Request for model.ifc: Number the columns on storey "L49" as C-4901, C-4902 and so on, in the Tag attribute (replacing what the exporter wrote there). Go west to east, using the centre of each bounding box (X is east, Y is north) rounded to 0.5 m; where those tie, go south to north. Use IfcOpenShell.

First a look at what the model holds.

```python
import ifcopenshell
import ifcopenshell.util.element
import ifcopenshell.util.placement

model = ifcopenshell.open("model.ifc")
print(model.schema)
storey = next(s for s in model.by_type("IfcBuildingStorey") if s.Name == "L49")
columns = [e for e in ifcopenshell.util.element.get_decomposition(storey) if e.is_a("IfcColumn")]
for e in sorted(columns, key=lambda e: e.id()):
    origin = ifcopenshell.util.placement.get_local_placement(e.ObjectPlacement)[:3, 3]
    print(e.id(), e.Tag, e.Name, origin.round(2) + 0.0, sep=" | ")
```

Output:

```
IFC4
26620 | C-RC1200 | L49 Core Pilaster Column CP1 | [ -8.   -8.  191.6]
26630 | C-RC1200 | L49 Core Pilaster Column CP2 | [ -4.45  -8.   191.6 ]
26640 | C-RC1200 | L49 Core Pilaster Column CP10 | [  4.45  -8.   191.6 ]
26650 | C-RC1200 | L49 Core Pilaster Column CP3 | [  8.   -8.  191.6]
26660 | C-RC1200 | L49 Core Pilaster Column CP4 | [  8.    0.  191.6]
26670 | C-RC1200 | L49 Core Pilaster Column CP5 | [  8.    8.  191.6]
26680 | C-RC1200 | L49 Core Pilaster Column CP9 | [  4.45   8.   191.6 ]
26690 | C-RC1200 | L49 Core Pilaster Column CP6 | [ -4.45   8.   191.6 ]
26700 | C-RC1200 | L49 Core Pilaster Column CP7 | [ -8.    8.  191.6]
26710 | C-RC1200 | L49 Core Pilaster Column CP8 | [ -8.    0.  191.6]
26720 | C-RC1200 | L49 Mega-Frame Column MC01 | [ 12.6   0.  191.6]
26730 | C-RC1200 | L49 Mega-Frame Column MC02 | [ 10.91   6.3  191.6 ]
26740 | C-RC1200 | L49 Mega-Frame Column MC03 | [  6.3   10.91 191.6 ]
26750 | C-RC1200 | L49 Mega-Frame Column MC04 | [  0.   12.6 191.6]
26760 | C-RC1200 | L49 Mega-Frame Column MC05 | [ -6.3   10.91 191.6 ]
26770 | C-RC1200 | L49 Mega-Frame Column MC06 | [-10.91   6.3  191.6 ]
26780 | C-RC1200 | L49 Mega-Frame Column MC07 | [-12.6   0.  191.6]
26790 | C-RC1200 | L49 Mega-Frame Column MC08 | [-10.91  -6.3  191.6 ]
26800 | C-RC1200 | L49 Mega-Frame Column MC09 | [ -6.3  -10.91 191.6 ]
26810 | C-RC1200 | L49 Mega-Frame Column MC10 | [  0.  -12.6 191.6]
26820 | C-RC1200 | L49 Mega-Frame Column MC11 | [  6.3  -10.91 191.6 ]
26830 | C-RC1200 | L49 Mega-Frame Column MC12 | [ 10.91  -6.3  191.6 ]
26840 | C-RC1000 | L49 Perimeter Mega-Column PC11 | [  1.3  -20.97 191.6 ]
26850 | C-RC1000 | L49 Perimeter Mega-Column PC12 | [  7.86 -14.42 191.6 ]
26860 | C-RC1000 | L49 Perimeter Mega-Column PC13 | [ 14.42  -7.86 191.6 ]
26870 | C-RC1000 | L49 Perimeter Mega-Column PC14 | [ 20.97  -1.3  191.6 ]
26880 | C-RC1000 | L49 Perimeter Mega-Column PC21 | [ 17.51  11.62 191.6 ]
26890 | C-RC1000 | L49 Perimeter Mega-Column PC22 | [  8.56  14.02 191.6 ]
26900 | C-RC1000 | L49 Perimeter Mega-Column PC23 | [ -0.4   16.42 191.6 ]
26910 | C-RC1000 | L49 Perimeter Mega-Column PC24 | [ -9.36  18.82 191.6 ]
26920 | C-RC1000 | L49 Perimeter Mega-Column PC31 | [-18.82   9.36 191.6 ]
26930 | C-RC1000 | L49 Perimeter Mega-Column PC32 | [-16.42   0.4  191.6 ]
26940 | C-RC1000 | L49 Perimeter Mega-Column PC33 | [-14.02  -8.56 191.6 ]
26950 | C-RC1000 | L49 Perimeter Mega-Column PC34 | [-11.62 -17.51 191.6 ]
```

```python
import ifcopenshell
import ifcopenshell.geom
import ifcopenshell.util.element
import ifcopenshell.util.shape

model = ifcopenshell.open("model.ifc")
settings = ifcopenshell.geom.settings()
settings.set("use-world-coords", True)


def centre(element):
    shape = ifcopenshell.geom.create_shape(settings, element)
    return ifcopenshell.util.shape.get_bbox_centroid(shape.geometry)


storey = next(s for s in model.by_type("IfcBuildingStorey") if s.Name == "L49")
columns = [e for e in ifcopenshell.util.element.get_decomposition(storey) if e.is_a("IfcColumn")]

# Insertion points can sit at a corner or the storey origin, so sort by the geometry (in metres).
centres = {e: centre(e) for e in columns}
columns.sort(key=lambda e: (round(centres[e][0] / 0.5), centres[e][1]))

for i, e in enumerate(columns, start=1):
    number = f"C-49{i:02d}"
    e.Tag = number
    print(e.id(), number)

model.write("model_updated.ifc")
```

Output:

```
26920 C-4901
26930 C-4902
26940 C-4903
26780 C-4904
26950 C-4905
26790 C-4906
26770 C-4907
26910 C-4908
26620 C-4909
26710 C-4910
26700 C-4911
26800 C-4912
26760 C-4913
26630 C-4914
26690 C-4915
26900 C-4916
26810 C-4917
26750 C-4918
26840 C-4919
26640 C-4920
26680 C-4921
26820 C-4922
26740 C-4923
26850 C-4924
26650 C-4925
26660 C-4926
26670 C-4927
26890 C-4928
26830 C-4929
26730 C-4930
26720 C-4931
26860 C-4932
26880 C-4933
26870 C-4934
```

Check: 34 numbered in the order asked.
